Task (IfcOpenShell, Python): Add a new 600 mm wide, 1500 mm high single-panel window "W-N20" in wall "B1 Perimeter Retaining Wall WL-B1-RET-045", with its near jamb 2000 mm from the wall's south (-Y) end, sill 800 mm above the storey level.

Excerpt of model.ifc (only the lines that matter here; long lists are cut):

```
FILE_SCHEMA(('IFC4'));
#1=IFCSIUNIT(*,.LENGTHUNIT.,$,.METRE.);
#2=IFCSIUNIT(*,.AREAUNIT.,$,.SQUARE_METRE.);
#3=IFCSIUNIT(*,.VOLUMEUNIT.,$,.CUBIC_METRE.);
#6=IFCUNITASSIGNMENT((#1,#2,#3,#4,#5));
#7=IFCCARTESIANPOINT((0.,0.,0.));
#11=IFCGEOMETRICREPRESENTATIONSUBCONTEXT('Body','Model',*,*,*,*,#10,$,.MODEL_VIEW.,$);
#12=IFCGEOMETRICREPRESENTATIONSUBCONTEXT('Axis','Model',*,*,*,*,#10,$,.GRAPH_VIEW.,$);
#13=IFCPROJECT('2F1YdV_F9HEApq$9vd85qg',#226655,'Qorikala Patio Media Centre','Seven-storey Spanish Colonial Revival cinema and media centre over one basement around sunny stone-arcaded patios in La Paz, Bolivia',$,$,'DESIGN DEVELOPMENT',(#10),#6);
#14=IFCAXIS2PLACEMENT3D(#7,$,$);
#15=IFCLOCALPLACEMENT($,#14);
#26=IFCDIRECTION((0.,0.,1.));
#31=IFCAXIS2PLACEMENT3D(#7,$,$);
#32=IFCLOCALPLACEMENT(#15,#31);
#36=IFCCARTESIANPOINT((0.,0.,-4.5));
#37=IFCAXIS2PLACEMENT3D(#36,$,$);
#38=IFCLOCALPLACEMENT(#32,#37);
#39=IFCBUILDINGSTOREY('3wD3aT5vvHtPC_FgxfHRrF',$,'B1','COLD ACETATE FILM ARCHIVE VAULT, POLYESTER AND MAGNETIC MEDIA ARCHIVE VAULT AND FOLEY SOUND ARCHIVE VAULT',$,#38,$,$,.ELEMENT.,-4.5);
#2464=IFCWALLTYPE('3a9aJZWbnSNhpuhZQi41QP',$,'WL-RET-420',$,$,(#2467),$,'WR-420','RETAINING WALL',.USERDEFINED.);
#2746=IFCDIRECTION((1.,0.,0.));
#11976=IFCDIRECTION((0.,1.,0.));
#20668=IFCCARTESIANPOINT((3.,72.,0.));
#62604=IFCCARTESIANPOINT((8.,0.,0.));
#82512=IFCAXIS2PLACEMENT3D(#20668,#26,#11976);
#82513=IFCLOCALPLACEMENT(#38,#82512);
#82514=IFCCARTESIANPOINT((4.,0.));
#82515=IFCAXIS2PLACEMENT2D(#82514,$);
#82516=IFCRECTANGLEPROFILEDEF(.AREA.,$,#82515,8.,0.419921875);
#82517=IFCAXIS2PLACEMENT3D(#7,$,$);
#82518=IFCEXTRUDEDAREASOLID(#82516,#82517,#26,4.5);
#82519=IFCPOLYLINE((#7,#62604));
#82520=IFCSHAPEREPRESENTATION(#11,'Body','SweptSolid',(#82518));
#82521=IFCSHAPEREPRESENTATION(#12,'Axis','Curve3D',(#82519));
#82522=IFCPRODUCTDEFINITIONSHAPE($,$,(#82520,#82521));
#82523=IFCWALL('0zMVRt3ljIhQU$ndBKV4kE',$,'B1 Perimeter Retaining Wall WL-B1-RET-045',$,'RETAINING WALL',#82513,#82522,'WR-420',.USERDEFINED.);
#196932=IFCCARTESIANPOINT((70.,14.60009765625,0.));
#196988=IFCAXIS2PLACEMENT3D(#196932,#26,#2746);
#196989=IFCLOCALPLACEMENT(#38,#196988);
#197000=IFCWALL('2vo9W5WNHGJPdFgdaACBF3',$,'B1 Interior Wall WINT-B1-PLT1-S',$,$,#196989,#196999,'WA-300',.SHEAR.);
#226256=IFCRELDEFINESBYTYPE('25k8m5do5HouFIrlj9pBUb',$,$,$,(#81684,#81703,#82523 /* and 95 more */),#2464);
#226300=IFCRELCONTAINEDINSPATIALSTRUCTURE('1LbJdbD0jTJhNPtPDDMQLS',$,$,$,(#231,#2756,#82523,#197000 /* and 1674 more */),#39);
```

```python
import numpy as np
import ifcopenshell
import ifcopenshell.api.feature
import ifcopenshell.api.geometry
import ifcopenshell.api.root
import ifcopenshell.api.spatial
import ifcopenshell.geom
import ifcopenshell.util.element
import ifcopenshell.util.placement
import ifcopenshell.util.representation
import ifcopenshell.util.shape
import ifcopenshell.util.unit

model = ifcopenshell.open("model.ifc")
unit_scale = ifcopenshell.util.unit.calculate_unit_scale(model)
settings = ifcopenshell.geom.settings()


def volume(element):
    """Net volume in cubic metres, openings subtracted."""
    shape = ifcopenshell.geom.create_shape(settings, element)
    return ifcopenshell.util.shape.get_volume(shape.geometry)


wall = model.by_id(82523)
storey = ifcopenshell.util.element.get_container(wall, ifc_class="IfcBuildingStorey")
context = ifcopenshell.util.representation.get_context(model, "Model", "Body", "MODEL_VIEW")
before = volume(wall)

width, height, from_end, sill = 0.6, 1.5, 2, 0.8  # metres

# The wall runs along its own X axis, and the end named is its -X end.
wall_shape = ifcopenshell.geom.create_shape(settings, wall)
x, y, z = ifcopenshell.util.shape.get_vertices(wall_shape.geometry).T
start = x.min() + from_end
face, thickness = float(y.min()), float(y.max() - y.min())
wall_matrix = ifcopenshell.util.placement.get_local_placement(wall.ObjectPlacement)
level = ifcopenshell.util.placement.get_local_placement(storey.ObjectPlacement)[2, 3]


def in_wall(x, y):
    """Placement at x, y metres in the wall's axes, at sill height."""
    matrix = wall_matrix.copy()
    matrix[:, 3] = wall_matrix @ np.array([x / unit_scale, y / unit_scale, 0.0, 1.0])
    matrix[2, 3] = level + sill / unit_scale
    return matrix


# Opening: a box that overshoots both wall faces by 50 mm.
opening = ifcopenshell.api.root.create_entity(model, ifc_class="IfcOpeningElement", predefined_type="OPENING")
box = ifcopenshell.api.geometry.add_wall_representation(
    model, context=context, length=width, height=height, thickness=thickness + 0.1
)
ifcopenshell.api.geometry.assign_representation(model, product=opening, representation=box)
ifcopenshell.api.geometry.edit_object_placement(model, product=opening, matrix=in_wall(start, face - 0.05), is_si=False)
ifcopenshell.api.feature.add_feature(model, feature=opening, element=wall)

window = ifcopenshell.api.root.create_entity(model, ifc_class="IfcWindow", name="W-N20", predefined_type="WINDOW")
window.OverallWidth, window.OverallHeight = width / unit_scale, height / unit_scale
window.PartitioningType = "SINGLE_PANEL"
body = ifcopenshell.api.geometry.add_window_representation(
    model,
    context=context,
    overall_width=window.OverallWidth,
    overall_height=window.OverallHeight,
    partition_type="SINGLE_PANEL",
)
ifcopenshell.api.geometry.assign_representation(model, product=window, representation=body)
ifcopenshell.api.spatial.assign_container(model, products=[window], relating_structure=storey)
ifcopenshell.api.feature.add_filling(model, opening=opening, element=window)

# Centre the window in the wall's thickness.
ifcopenshell.api.geometry.edit_object_placement(model, product=window, matrix=in_wall(start, face), is_si=False)
window_shape = ifcopenshell.geom.create_shape(settings, window)
depth = ifcopenshell.util.shape.get_vertices(window_shape.geometry)[:, 1]
offset = face + thickness / 2 - (depth.min() + depth.max()) / 2
ifcopenshell.api.geometry.edit_object_placement(model, product=window, matrix=in_wall(start, offset), is_si=False)

after = volume(wall)

print(f"wall volume {before:.3f} -> {after:.3f} m3")

model.write("model_edited.ifc")
```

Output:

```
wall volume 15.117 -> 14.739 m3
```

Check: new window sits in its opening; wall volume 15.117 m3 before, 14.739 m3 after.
